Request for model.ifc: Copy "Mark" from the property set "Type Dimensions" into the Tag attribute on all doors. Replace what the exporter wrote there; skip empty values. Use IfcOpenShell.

First a look at what the model holds.

```python
import ifcopenshell
import ifcopenshell.util.element

model = ifcopenshell.open("model.ifc")
print(model.schema)
doors = model.by_type("IfcDoor")
print(len(doors), "doors")
for e in doors[:8]:
    source = ifcopenshell.util.element.get_pset(e, "Type Dimensions", "Mark")
    target = e.Tag
    print(e.id(), repr(source), repr(target), sep=" | ")
```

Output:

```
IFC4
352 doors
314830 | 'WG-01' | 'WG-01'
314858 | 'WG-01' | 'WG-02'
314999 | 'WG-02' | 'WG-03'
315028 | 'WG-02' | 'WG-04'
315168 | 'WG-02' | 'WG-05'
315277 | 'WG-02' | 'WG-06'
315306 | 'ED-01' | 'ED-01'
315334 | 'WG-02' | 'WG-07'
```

```python
import ifcopenshell
import ifcopenshell.util.element

model = ifcopenshell.open("model.ifc")

count = 0
for e in model.by_type("IfcDoor"):
    value = ifcopenshell.util.element.get_pset(e, "Type Dimensions", "Mark")
    current = e.Tag
    if not value or not value.strip() or current == value:
        continue
    e.Tag = value
    count += 1

print(count, "doors updated")

model.write("model_edited.ifc")
```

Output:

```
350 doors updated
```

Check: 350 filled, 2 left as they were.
